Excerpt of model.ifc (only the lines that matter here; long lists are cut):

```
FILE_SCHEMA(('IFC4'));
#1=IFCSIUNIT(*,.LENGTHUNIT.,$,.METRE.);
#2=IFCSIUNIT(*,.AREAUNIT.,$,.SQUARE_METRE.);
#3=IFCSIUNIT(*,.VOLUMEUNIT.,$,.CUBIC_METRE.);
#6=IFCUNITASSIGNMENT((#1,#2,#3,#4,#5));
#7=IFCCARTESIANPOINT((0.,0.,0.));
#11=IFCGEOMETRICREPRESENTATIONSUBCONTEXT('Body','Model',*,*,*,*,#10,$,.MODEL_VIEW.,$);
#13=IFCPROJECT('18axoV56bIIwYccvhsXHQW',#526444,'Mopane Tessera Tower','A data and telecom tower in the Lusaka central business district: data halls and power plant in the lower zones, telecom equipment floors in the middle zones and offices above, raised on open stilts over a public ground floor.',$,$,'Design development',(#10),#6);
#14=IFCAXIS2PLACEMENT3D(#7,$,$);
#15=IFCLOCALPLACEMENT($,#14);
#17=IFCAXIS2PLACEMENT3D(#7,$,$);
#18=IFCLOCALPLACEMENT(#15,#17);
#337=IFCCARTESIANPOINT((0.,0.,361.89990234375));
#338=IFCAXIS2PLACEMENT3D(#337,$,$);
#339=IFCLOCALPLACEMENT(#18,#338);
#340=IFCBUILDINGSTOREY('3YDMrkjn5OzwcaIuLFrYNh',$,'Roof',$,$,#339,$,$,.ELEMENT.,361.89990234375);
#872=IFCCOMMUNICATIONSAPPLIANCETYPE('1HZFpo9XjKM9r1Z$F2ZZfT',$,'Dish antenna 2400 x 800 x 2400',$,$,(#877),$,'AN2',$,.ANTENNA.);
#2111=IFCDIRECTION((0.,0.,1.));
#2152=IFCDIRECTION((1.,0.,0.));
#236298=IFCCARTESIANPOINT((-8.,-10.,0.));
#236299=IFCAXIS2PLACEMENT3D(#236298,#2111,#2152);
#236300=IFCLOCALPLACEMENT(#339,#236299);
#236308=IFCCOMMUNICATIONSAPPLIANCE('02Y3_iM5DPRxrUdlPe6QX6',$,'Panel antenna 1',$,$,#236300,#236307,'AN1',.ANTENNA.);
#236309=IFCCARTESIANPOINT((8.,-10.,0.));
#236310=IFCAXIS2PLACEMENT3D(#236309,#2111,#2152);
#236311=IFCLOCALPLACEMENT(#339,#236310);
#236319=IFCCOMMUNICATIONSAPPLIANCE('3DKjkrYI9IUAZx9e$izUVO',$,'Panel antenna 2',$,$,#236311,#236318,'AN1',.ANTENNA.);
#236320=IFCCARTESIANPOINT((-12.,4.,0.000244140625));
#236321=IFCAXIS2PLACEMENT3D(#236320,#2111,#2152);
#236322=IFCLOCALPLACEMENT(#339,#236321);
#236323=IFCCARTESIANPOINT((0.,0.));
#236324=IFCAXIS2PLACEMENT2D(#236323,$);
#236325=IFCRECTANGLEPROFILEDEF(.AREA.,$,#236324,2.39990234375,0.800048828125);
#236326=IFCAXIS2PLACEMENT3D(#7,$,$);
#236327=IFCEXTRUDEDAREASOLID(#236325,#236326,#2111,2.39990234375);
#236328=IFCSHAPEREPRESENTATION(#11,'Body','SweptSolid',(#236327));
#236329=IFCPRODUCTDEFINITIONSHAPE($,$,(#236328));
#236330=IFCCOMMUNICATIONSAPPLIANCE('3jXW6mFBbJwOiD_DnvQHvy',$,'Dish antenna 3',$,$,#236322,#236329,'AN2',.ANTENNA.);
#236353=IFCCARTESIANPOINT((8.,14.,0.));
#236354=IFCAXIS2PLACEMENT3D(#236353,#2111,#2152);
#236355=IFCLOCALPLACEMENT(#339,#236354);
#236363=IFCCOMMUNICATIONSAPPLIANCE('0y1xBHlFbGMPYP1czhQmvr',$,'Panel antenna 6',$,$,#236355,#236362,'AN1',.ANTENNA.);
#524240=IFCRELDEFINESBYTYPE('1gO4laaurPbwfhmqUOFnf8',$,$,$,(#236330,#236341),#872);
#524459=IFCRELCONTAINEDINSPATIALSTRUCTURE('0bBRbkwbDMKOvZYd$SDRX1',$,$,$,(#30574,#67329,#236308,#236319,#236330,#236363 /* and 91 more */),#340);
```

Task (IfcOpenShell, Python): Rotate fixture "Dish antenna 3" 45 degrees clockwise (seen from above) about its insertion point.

```python
import ifcopenshell
import ifcopenshell.api.geometry
import ifcopenshell.util.placement

model = ifcopenshell.open("model.ifc")

item = model.by_id(236330)
matrix = ifcopenshell.util.placement.get_local_placement(item.ObjectPlacement)
matrix = matrix @ ifcopenshell.util.placement.rotation(-45, "Z")
ifcopenshell.api.geometry.edit_object_placement(model, product=item, matrix=matrix, is_si=False)

print(ifcopenshell.util.placement.get_local_placement(item.ObjectPlacement).round(3) + 0.0)

model.write("model_rev.ifc")
```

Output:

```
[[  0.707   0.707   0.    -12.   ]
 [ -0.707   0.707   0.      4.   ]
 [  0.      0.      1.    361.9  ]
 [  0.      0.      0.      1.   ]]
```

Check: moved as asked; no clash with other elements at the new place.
